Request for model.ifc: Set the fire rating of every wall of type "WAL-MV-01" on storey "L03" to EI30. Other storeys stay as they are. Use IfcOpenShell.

First a look at what the model holds.

```python
import ifcopenshell
import ifcopenshell.util.element

model = ifcopenshell.open("model.ifc")
print(model.schema)
storey = next(s for s in model.by_type("IfcBuildingStorey") if s.Name == "L03")
walls = [e for e in ifcopenshell.util.element.get_decomposition(storey) if e.is_a("IfcWall")]
seen = {}
for e in walls:
    element_type = ifcopenshell.util.element.get_type(e)
    key = (element_type.Name if element_type != e and element_type else None, ifcopenshell.util.element.get_pset(e, "Pset_WallCommon", "FireRating"))
    seen[key] = seen.get(key, 0) + 1
for (name, value), count in sorted(seen.items(), key=str):
    print(count, "x", name, "|", value)
```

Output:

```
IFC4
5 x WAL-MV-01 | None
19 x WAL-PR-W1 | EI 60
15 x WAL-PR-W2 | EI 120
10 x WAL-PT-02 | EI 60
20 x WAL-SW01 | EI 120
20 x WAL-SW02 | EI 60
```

```python
import ifcopenshell
import ifcopenshell.api.pset
import ifcopenshell.util.element

model = ifcopenshell.open("model.ifc")

storey = next(s for s in model.by_type("IfcBuildingStorey") if s.Name == "L03")
walls = [e for e in ifcopenshell.util.element.get_decomposition(storey) if e.is_a("IfcWall")]

count = 0
for e in walls:
    element_type = ifcopenshell.util.element.get_type(e)
    if element_type in (None, e) or element_type.Name != "WAL-MV-01":
        continue
    # add_pset returns the element's existing set when there is one.
    pset = ifcopenshell.api.pset.add_pset(model, product=e, name="Pset_WallCommon")
    ifcopenshell.api.pset.edit_pset(model, pset=pset, properties={"FireRating": "EI30"})
    count += 1

print(count, "walls updated")

model.write("model_updated.ifc")
```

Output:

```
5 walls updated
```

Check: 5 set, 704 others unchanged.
